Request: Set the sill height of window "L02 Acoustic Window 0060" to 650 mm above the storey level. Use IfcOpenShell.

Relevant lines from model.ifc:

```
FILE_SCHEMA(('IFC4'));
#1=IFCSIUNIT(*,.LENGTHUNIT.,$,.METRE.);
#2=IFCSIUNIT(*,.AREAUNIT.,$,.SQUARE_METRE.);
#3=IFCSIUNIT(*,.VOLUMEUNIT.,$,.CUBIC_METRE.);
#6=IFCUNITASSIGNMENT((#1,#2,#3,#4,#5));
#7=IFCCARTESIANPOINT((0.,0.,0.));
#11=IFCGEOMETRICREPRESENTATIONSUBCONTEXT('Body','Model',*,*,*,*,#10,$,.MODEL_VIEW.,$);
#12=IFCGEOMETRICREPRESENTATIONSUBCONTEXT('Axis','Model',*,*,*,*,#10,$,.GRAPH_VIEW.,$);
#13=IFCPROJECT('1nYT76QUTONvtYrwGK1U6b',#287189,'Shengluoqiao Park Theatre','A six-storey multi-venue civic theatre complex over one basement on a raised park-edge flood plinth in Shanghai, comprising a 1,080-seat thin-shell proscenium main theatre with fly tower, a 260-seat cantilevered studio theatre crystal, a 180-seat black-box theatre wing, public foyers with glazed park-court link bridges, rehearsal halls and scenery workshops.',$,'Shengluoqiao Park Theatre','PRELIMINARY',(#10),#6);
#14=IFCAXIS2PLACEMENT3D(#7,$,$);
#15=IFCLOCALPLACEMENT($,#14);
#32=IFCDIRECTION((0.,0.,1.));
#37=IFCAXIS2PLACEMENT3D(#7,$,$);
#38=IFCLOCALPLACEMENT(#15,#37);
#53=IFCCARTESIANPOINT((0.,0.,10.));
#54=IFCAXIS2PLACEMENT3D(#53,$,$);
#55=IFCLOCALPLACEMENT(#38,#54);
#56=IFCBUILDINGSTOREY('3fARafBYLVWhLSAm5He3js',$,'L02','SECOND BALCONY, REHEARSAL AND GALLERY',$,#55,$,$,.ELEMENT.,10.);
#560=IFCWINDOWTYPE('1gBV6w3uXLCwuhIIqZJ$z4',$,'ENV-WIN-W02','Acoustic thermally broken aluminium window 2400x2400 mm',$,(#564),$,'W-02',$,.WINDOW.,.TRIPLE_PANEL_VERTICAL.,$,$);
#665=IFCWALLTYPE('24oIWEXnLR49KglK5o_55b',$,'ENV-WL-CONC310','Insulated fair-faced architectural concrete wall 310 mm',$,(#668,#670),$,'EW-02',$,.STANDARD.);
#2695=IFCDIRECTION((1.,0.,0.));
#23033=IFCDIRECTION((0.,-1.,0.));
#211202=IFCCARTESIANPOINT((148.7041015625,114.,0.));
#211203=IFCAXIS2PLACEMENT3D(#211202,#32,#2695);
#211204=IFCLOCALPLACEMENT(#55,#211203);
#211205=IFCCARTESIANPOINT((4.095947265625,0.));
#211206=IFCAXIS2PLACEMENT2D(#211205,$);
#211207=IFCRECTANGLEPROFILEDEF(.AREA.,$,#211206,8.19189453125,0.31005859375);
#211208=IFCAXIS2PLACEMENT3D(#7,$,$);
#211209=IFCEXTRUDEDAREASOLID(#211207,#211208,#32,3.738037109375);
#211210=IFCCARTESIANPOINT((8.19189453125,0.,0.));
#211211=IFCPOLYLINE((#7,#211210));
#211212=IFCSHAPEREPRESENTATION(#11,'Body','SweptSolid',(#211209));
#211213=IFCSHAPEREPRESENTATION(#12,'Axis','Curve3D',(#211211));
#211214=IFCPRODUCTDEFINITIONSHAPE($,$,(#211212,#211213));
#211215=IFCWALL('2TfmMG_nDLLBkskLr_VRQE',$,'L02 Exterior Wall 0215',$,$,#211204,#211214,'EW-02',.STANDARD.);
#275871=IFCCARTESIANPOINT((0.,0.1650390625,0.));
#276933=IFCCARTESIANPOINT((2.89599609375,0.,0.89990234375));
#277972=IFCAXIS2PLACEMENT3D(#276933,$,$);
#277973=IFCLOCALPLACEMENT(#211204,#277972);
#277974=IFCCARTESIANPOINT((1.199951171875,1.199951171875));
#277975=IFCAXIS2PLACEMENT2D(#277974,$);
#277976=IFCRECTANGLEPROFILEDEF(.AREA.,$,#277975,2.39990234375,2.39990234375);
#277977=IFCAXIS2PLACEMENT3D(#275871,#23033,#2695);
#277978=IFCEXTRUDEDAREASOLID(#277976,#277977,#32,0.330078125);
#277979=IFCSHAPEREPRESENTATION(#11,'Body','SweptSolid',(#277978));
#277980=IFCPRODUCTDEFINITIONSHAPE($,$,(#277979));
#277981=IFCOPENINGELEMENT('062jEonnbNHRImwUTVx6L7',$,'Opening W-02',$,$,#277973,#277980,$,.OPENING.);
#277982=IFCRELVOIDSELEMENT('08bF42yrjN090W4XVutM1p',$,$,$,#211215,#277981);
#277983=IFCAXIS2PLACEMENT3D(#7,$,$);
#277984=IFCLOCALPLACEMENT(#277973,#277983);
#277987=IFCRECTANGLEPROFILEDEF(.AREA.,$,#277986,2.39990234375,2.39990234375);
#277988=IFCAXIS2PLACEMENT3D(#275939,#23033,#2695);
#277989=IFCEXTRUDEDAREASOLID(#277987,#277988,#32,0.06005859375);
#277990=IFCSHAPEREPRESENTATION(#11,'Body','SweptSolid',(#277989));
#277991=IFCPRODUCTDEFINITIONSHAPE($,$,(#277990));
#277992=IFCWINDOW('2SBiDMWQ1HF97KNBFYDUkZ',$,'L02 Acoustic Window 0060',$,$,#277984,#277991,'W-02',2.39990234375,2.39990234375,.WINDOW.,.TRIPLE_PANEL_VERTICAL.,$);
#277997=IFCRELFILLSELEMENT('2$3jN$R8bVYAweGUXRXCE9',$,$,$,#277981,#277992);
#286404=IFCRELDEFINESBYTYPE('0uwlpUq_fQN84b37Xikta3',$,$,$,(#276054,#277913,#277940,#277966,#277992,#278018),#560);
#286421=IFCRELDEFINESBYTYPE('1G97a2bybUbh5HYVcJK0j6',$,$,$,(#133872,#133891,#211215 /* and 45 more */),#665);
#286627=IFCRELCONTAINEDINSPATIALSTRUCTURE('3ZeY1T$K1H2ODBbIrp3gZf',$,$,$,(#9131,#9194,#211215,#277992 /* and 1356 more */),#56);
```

```python
import numpy as np
import ifcopenshell
import ifcopenshell.api.geometry
import ifcopenshell.geom
import ifcopenshell.util.element
import ifcopenshell.util.placement
import ifcopenshell.util.shape
import ifcopenshell.util.unit

model = ifcopenshell.open("model.ifc")
unit_scale = ifcopenshell.util.unit.calculate_unit_scale(model)

window = model.by_id(277992)
opening = window.FillsVoids[0].RelatingOpeningElement
storey = ifcopenshell.util.element.get_container(window, ifc_class="IfcBuildingStorey")
level = ifcopenshell.util.placement.get_local_placement(storey.ObjectPlacement)[2, 3]

# The opening's origin need not be at the sill, so measure its lowest point.
shape = ifcopenshell.geom.create_shape(ifcopenshell.geom.settings(), opening)
bottom = ifcopenshell.util.shape.get_shape_bottom_elevation(shape, shape.geometry) / unit_scale
dz = level + 0.65 - bottom

shift = np.array([0.0, 0.0, dz])
# The window is placed relative to its opening, so it follows when the opening moves.
matrix = ifcopenshell.util.placement.get_local_placement(opening.ObjectPlacement)
matrix[:3, 3] += shift
ifcopenshell.api.geometry.edit_object_placement(
    model, product=opening, matrix=matrix, is_si=False, should_transform_children=True
)

print(f"moved by {dz * unit_scale:+.3f} m")

model.write("model_edited.ifc")
```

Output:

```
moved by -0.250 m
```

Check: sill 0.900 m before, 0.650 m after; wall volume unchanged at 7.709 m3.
